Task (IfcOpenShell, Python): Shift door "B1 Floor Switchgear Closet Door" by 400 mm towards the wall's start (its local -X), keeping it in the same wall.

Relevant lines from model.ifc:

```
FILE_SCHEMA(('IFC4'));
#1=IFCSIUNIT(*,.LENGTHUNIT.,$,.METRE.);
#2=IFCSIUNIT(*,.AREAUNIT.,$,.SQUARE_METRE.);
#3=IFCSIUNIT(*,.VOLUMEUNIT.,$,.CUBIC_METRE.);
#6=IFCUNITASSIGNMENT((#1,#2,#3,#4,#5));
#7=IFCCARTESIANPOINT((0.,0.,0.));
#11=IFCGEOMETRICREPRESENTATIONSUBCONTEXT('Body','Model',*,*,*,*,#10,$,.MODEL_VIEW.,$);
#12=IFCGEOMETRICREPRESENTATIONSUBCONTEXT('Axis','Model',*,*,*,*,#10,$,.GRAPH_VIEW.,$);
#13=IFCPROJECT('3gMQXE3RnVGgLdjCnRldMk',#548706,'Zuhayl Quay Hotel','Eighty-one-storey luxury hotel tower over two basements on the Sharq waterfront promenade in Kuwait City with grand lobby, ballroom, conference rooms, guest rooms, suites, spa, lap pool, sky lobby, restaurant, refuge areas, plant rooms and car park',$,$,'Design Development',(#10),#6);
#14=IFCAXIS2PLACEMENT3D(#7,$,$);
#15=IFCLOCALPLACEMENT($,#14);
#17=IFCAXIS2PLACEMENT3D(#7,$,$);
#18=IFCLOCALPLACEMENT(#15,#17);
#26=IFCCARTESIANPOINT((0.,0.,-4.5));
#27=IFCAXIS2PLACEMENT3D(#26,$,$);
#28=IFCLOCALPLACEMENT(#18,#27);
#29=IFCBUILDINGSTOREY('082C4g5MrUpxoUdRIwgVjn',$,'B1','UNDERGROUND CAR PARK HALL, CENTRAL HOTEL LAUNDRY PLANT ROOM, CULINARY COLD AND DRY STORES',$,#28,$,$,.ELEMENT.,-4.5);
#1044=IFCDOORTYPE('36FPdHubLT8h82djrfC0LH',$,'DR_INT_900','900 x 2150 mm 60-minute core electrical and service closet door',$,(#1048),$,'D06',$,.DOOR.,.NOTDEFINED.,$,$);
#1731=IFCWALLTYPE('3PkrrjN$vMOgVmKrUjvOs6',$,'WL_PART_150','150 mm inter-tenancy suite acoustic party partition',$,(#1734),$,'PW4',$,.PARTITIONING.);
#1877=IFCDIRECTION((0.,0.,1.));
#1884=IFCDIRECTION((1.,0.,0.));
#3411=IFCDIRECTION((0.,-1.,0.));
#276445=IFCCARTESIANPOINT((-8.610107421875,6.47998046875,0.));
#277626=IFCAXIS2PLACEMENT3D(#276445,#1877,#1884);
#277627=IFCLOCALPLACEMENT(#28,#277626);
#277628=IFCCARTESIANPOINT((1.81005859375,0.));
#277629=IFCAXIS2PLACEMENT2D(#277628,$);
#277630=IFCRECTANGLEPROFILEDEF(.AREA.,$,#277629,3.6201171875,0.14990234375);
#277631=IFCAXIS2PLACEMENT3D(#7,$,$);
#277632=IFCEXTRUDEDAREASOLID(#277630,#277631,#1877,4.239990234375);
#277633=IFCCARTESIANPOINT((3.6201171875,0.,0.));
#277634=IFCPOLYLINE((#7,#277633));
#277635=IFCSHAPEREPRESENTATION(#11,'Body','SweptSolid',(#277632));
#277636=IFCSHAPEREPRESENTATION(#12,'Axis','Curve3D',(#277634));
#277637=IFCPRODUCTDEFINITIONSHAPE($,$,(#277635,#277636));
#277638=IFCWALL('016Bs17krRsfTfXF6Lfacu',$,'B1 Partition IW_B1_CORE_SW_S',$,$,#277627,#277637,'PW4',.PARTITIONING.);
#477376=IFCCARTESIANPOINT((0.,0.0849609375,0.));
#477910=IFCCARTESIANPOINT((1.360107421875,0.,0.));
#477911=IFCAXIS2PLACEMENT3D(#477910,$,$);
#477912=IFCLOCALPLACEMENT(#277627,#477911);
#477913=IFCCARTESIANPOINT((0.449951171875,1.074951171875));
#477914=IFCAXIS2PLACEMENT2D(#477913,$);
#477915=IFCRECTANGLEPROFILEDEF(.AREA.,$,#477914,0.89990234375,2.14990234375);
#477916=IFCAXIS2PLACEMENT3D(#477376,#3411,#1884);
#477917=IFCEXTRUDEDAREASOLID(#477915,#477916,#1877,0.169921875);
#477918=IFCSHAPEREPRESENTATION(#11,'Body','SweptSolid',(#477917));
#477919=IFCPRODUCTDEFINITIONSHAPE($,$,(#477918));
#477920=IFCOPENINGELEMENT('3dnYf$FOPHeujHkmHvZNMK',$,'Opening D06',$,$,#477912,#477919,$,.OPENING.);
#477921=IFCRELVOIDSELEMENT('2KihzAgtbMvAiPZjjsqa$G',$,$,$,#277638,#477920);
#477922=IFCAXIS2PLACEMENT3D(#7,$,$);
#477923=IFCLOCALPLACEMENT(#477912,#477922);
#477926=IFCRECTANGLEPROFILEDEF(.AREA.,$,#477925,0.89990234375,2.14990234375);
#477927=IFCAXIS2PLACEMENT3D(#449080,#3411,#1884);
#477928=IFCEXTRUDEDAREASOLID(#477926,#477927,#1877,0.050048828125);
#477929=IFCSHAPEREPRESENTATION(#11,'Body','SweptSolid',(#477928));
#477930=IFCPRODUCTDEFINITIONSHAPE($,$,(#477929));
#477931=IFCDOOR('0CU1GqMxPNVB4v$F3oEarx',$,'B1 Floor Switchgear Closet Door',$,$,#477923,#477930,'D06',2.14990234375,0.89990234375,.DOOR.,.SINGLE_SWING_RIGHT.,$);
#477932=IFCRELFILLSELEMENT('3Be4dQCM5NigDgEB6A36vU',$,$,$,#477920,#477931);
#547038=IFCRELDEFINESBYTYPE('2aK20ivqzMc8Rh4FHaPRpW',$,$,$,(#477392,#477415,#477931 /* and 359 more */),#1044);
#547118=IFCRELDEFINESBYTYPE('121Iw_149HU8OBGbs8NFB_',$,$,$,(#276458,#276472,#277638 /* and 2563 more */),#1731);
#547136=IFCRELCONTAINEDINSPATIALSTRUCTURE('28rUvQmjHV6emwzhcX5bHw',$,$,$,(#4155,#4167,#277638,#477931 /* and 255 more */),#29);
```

```python
import ifcopenshell
import ifcopenshell.api.geometry
import ifcopenshell.util.placement
import ifcopenshell.util.unit

model = ifcopenshell.open("model.ifc")
unit_scale = ifcopenshell.util.unit.calculate_unit_scale(model)

door = model.by_guid("0CU1GqMxPNVB4v$F3oEarx")
opening = door.FillsVoids[0].RelatingOpeningElement
wall = opening.VoidsElements[0].RelatingBuildingElement

wall_matrix = ifcopenshell.util.placement.get_local_placement(wall.ObjectPlacement)
shift = wall_matrix[:3, 0] * -0.4 / unit_scale
before = ifcopenshell.util.placement.get_local_placement(door.ObjectPlacement)[:3, 3].copy()

# The door is placed relative to its opening, so it follows when the opening moves.
matrix = ifcopenshell.util.placement.get_local_placement(opening.ObjectPlacement)
matrix[:3, 3] += shift
ifcopenshell.api.geometry.edit_object_placement(
    model, product=opening, matrix=matrix, is_si=False, should_transform_children=True
)

after = ifcopenshell.util.placement.get_local_placement(door.ObjectPlacement)[:3, 3]
print("door moved by", (after - before).round(3) + 0.0)

model.write("model-out.ifc")
```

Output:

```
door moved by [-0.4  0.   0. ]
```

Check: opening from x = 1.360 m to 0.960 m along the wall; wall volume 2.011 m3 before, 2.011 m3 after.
